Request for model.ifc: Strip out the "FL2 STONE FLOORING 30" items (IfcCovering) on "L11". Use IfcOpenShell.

First a look at what the model holds.

```python
import ifcopenshell
import ifcopenshell.util.element

model = ifcopenshell.open("model.ifc")
print(model.schema)
storey = next(s for s in model.by_type("IfcBuildingStorey") if s.Name == "L11")
coverings = [e for e in ifcopenshell.util.element.get_decomposition(storey) if e.is_a("IfcCovering")]
seen = {}
for e in coverings:
    element_type = ifcopenshell.util.element.get_type(e)
    name = element_type.Name if element_type not in (None, e) else None
    seen[name] = seen.get(name, 0) + 1
for name, count in sorted(seen.items(), key=str):
    print(count, "x", name)
```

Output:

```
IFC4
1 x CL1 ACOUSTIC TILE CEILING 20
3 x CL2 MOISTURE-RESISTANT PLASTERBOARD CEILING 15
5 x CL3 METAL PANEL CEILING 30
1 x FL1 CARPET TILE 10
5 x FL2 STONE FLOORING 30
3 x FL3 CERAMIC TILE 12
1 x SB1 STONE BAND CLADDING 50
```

```python
import ifcopenshell
import ifcopenshell.api.root
import ifcopenshell.util.element

model = ifcopenshell.open("model.ifc")

storey = next(s for s in model.by_type("IfcBuildingStorey") if s.Name == "L11")
coverings = [e for e in ifcopenshell.util.element.get_decomposition(storey) if e.is_a("IfcCovering")]
targets = [e for e in coverings if (t := ifcopenshell.util.element.get_type(e)) not in (None, e) and t.Name == "FL2 STONE FLOORING 30"]

for e in targets:
    ifcopenshell.api.root.remove_product(model, product=e)
print(len(targets), "removed")

model.write("model_edited.ifc")
```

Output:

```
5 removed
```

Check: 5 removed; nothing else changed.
